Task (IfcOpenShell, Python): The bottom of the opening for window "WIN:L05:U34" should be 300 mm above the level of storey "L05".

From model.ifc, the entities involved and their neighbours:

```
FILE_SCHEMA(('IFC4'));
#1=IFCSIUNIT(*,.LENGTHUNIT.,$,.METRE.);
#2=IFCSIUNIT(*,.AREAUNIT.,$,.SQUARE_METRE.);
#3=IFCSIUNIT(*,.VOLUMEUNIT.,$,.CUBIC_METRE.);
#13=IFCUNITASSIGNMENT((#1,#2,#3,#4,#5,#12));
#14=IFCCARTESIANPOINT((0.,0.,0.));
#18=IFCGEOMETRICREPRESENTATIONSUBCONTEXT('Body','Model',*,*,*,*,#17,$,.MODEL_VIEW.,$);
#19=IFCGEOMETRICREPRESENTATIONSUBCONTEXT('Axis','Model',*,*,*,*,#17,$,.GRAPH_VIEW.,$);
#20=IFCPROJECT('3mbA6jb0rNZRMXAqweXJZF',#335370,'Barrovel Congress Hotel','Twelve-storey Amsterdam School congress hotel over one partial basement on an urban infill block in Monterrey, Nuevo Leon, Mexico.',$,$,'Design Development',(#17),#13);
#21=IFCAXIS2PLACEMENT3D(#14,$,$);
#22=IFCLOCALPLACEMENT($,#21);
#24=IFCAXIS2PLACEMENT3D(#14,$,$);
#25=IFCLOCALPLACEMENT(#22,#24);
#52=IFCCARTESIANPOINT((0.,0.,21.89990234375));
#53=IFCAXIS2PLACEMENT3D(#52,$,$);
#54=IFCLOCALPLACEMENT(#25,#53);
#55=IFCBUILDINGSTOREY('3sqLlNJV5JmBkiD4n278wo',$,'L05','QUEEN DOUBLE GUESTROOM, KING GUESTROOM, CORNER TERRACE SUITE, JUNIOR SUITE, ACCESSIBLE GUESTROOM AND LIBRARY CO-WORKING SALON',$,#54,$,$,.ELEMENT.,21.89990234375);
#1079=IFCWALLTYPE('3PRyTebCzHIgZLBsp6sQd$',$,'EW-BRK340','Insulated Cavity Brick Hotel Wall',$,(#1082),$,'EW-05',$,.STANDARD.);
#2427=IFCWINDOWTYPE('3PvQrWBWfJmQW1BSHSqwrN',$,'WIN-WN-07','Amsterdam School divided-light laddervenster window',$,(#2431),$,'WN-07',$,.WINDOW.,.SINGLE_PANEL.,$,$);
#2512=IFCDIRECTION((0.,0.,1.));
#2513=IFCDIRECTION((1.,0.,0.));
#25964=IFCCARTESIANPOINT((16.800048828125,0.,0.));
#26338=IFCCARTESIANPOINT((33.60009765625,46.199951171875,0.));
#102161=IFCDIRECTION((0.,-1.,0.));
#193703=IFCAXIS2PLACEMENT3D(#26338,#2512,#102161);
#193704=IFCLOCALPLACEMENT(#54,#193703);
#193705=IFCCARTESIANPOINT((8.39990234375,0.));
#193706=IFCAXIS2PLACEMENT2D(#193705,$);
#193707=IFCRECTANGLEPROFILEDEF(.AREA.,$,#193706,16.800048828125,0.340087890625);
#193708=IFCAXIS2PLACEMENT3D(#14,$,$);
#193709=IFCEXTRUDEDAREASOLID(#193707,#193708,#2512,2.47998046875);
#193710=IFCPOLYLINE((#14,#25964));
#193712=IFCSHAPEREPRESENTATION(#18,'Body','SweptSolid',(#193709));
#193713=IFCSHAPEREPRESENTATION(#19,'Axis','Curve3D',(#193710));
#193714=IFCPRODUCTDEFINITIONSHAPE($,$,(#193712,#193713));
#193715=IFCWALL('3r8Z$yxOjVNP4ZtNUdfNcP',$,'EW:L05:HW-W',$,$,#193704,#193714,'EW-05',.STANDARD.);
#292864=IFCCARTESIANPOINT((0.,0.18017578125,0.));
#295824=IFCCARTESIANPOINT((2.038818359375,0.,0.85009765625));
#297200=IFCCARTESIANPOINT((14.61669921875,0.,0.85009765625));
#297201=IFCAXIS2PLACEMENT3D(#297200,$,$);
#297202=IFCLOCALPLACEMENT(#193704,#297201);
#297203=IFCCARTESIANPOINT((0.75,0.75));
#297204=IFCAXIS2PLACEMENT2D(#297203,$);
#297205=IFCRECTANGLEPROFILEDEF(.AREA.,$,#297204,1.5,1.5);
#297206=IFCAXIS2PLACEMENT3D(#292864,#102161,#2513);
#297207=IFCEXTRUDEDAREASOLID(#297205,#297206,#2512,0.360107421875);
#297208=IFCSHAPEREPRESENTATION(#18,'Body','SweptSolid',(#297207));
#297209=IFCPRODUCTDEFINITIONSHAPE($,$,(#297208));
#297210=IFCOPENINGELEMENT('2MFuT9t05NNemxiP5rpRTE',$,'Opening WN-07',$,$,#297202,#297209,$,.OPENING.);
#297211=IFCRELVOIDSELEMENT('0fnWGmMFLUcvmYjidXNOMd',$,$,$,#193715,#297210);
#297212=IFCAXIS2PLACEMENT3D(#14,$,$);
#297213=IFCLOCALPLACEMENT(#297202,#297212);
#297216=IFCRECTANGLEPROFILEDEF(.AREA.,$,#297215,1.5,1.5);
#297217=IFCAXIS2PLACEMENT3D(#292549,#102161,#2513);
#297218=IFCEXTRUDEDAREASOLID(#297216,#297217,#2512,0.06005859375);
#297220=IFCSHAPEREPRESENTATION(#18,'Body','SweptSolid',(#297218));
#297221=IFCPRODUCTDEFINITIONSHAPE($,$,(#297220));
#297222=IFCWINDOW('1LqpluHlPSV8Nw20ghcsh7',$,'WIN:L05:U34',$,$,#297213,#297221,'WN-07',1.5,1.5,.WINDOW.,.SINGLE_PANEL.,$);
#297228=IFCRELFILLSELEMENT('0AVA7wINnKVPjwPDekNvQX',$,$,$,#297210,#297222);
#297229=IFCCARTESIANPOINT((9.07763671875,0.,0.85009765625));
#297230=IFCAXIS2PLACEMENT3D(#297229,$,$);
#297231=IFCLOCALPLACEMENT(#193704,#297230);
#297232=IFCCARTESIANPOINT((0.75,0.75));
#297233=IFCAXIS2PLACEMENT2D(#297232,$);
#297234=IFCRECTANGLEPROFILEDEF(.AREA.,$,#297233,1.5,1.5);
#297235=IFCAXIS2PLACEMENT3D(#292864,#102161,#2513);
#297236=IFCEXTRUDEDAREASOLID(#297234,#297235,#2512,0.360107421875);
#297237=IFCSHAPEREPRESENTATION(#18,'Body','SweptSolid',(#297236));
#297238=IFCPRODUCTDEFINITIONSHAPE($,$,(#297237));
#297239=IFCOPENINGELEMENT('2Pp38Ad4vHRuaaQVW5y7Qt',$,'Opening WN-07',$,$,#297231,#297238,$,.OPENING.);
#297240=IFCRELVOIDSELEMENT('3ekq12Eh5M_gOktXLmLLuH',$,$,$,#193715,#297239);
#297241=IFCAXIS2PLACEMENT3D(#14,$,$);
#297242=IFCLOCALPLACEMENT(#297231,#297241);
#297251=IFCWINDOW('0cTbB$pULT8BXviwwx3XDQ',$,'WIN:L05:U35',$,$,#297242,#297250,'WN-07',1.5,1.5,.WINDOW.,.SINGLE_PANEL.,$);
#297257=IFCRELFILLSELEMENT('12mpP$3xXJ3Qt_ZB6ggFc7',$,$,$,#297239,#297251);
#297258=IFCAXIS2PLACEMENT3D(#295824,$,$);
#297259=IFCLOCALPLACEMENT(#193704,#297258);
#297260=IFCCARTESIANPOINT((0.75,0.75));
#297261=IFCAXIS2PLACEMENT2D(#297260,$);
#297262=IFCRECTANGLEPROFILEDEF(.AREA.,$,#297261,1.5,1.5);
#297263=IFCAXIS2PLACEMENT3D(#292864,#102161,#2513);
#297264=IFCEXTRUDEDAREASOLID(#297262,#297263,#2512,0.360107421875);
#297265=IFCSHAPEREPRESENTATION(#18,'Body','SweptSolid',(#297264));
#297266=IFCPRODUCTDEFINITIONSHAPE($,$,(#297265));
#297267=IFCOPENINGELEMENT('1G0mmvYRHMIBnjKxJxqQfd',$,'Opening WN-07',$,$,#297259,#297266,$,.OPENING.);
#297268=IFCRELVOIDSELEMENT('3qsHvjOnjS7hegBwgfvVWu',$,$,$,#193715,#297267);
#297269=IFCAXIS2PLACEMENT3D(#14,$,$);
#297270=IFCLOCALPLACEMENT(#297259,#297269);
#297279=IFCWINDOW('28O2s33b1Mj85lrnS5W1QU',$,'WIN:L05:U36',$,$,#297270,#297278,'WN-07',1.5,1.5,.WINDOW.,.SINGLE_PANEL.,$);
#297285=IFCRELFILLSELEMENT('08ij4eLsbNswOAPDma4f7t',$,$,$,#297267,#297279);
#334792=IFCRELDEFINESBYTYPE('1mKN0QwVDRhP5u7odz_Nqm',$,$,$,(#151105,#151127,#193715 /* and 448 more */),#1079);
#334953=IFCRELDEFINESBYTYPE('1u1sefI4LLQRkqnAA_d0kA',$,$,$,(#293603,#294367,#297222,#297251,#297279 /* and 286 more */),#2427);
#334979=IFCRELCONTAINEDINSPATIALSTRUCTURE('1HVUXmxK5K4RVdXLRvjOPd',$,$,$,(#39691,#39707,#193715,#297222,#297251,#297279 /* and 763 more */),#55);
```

```python
import numpy as np
import ifcopenshell
import ifcopenshell.api.geometry
import ifcopenshell.geom
import ifcopenshell.util.element
import ifcopenshell.util.placement
import ifcopenshell.util.shape
import ifcopenshell.util.unit

model = ifcopenshell.open("model.ifc")
unit_scale = ifcopenshell.util.unit.calculate_unit_scale(model)

window = model.by_guid("1LqpluHlPSV8Nw20ghcsh7")
opening = window.FillsVoids[0].RelatingOpeningElement
storey = ifcopenshell.util.element.get_container(window, ifc_class="IfcBuildingStorey")
level = ifcopenshell.util.placement.get_local_placement(storey.ObjectPlacement)[2, 3]

# The opening's origin need not be at the sill, so measure its lowest point.
shape = ifcopenshell.geom.create_shape(ifcopenshell.geom.settings(), opening)
bottom = ifcopenshell.util.shape.get_shape_bottom_elevation(shape, shape.geometry) / unit_scale
dz = level + 0.3 - bottom

shift = np.array([0.0, 0.0, dz])
# The window is placed relative to its opening, so it follows when the opening moves.
matrix = ifcopenshell.util.placement.get_local_placement(opening.ObjectPlacement)
matrix[:3, 3] += shift
ifcopenshell.api.geometry.edit_object_placement(
    model, product=opening, matrix=matrix, is_si=False, should_transform_children=True
)

print(f"moved by {dz * unit_scale:+.3f} m")

model.write("model_edited.ifc")
```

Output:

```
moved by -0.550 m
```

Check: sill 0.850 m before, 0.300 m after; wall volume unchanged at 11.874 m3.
